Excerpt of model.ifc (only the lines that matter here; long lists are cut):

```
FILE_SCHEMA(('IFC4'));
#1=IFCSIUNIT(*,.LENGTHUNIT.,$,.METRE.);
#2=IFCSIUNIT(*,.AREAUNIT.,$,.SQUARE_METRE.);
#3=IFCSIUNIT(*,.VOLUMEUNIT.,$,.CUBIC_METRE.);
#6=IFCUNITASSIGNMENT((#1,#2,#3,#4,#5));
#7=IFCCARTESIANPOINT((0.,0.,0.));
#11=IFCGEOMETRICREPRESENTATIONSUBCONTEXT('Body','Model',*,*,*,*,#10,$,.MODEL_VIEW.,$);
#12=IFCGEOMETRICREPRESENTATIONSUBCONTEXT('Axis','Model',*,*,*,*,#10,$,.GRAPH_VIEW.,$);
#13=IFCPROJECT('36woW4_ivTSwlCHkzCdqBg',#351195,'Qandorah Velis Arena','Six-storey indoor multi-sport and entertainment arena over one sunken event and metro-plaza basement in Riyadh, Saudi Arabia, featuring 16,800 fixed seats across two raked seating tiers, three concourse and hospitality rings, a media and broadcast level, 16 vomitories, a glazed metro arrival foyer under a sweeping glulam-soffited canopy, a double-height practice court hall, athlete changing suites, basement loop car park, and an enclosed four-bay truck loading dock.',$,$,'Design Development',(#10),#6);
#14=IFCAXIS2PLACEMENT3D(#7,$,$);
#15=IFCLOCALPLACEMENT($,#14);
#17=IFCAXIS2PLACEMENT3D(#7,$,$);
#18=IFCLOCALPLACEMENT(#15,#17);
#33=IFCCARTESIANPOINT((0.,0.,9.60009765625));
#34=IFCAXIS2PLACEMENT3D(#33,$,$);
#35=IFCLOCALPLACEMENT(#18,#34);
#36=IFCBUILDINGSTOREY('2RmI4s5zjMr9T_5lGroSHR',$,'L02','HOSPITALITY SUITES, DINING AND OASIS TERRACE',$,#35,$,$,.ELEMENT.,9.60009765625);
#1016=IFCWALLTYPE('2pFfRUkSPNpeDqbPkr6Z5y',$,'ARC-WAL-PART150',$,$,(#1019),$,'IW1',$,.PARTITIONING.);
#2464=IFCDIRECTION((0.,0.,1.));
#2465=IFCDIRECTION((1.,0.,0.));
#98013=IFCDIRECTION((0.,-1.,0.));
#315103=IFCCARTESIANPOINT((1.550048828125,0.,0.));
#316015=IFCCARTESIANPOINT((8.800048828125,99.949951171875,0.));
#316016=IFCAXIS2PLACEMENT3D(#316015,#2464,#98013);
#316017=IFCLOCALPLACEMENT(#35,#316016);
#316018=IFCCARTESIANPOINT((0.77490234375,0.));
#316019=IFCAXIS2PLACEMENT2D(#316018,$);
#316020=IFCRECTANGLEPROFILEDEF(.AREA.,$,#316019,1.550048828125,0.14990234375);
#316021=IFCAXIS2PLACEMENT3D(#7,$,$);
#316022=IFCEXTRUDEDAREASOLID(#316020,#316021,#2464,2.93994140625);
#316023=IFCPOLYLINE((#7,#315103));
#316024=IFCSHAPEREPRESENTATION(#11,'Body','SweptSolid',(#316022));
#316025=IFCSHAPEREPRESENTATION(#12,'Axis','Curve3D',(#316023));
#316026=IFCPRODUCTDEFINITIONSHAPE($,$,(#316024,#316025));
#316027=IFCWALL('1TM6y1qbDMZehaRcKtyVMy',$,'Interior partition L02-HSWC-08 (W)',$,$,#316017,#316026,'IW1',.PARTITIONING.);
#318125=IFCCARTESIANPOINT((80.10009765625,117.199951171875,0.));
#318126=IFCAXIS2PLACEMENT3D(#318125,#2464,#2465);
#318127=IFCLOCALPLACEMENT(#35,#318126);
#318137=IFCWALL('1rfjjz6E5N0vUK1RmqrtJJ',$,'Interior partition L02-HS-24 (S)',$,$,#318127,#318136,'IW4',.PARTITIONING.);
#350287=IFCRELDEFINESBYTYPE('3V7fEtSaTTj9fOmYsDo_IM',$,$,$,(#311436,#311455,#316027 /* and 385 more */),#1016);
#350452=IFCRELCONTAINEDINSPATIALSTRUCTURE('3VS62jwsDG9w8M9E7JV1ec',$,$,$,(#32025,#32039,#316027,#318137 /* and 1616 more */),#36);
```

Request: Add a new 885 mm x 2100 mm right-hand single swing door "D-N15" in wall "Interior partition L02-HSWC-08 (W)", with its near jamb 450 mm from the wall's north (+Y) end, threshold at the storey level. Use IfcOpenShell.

```python
import numpy as np
import ifcopenshell
import ifcopenshell.api.feature
import ifcopenshell.api.geometry
import ifcopenshell.api.root
import ifcopenshell.api.spatial
import ifcopenshell.geom
import ifcopenshell.util.element
import ifcopenshell.util.placement
import ifcopenshell.util.representation
import ifcopenshell.util.shape
import ifcopenshell.util.unit

model = ifcopenshell.open("model.ifc")
unit_scale = ifcopenshell.util.unit.calculate_unit_scale(model)
settings = ifcopenshell.geom.settings()


def volume(element):
    """Net volume in cubic metres, openings subtracted."""
    shape = ifcopenshell.geom.create_shape(settings, element)
    return ifcopenshell.util.shape.get_volume(shape.geometry)


wall = model.by_guid("1TM6y1qbDMZehaRcKtyVMy")
storey = ifcopenshell.util.element.get_container(wall, ifc_class="IfcBuildingStorey")
context = ifcopenshell.util.representation.get_context(model, "Model", "Body", "MODEL_VIEW")
before = volume(wall)

width, height, from_end, sill = 0.885, 2.1, 0.45, 0.0  # metres

# The wall runs along its own X axis, and the end named is its -X end.
wall_shape = ifcopenshell.geom.create_shape(settings, wall)
x, y, z = ifcopenshell.util.shape.get_vertices(wall_shape.geometry).T
start = x.min() + from_end
face, thickness = float(y.min()), float(y.max() - y.min())
wall_matrix = ifcopenshell.util.placement.get_local_placement(wall.ObjectPlacement)
level = ifcopenshell.util.placement.get_local_placement(storey.ObjectPlacement)[2, 3]


def in_wall(x, y):
    """Placement at x, y metres in the wall's axes, at sill height."""
    matrix = wall_matrix.copy()
    matrix[:, 3] = wall_matrix @ np.array([x / unit_scale, y / unit_scale, 0.0, 1.0])
    matrix[2, 3] = level + sill / unit_scale
    return matrix


# Opening: a box that overshoots both wall faces by 50 mm.
opening = ifcopenshell.api.root.create_entity(model, ifc_class="IfcOpeningElement", predefined_type="OPENING")
box = ifcopenshell.api.geometry.add_wall_representation(
    model, context=context, length=width, height=height, thickness=thickness + 0.1
)
ifcopenshell.api.geometry.assign_representation(model, product=opening, representation=box)
ifcopenshell.api.geometry.edit_object_placement(model, product=opening, matrix=in_wall(start, face - 0.05), is_si=False)
ifcopenshell.api.feature.add_feature(model, feature=opening, element=wall)

door = ifcopenshell.api.root.create_entity(model, ifc_class="IfcDoor", name="D-N15", predefined_type="DOOR")
door.OverallWidth, door.OverallHeight = width / unit_scale, height / unit_scale
door.OperationType = "SINGLE_SWING_RIGHT"
body = ifcopenshell.api.geometry.add_door_representation(
    model,
    context=context,
    overall_width=door.OverallWidth,
    overall_height=door.OverallHeight,
    operation_type="SINGLE_SWING_RIGHT",
    lining_properties={"LiningDepth": thickness / unit_scale, "ThresholdDepth": thickness / unit_scale},
)
ifcopenshell.api.geometry.assign_representation(model, product=door, representation=body)
ifcopenshell.api.spatial.assign_container(model, products=[door], relating_structure=storey)
ifcopenshell.api.feature.add_filling(model, opening=opening, element=door)

# The lining spans the wall, so the door starts at the wall face.
ifcopenshell.api.geometry.edit_object_placement(model, product=door, matrix=in_wall(start, face), is_si=False)

after = volume(wall)

print(f"wall volume {before:.3f} -> {after:.3f} m3")

model.write("model-out.ifc")
```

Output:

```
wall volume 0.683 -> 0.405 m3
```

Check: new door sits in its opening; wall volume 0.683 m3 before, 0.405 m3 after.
